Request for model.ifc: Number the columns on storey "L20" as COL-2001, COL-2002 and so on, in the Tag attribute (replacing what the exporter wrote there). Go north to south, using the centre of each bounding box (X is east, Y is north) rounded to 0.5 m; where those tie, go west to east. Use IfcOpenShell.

First a look at what the model holds.

```python
import ifcopenshell
import ifcopenshell.util.element
import ifcopenshell.util.placement

model = ifcopenshell.open("model.ifc")
print(model.schema)
storey = next(s for s in model.by_type("IfcBuildingStorey") if s.Name == "L20")
columns = [e for e in ifcopenshell.util.element.get_decomposition(storey) if e.is_a("IfcColumn")]
for e in sorted(columns, key=lambda e: e.id()):
    origin = ifcopenshell.util.placement.get_local_placement(e.ObjectPlacement)[:3, 3]
    print(e.id(), e.Tag, e.Name, origin.round(2) + 0.0, sep=" | ")
```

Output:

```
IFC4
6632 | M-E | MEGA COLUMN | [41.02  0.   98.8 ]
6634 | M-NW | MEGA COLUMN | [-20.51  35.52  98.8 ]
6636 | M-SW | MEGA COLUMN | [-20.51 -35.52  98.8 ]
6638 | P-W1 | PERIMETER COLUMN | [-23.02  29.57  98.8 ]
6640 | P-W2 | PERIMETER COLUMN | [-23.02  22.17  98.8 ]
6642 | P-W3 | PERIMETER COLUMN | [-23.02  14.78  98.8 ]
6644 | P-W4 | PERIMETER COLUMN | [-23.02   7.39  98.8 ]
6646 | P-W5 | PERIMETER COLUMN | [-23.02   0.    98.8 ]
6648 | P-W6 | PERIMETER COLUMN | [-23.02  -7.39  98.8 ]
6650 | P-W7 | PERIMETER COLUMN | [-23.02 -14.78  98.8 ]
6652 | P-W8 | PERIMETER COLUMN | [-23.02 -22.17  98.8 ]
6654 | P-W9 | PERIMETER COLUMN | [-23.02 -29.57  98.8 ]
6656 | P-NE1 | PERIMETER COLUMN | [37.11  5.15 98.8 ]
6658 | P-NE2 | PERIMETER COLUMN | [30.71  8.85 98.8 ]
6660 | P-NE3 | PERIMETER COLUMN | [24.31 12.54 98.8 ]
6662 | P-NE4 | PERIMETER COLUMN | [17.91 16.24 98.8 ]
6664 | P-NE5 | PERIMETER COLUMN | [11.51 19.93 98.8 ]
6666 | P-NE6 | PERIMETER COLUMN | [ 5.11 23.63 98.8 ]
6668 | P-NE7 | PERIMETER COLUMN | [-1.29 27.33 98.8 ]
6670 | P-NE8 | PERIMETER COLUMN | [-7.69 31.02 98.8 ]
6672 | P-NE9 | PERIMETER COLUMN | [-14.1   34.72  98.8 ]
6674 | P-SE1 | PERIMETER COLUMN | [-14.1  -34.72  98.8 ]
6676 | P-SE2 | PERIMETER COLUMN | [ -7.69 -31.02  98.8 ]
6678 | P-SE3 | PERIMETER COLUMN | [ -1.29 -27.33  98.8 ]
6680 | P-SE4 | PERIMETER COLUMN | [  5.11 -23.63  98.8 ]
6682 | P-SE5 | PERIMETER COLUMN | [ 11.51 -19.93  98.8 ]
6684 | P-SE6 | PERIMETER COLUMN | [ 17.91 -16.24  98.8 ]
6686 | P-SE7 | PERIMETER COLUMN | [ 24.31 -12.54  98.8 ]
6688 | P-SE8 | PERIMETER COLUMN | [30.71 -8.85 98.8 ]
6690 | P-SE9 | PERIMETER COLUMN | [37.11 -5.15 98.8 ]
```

```python
import ifcopenshell
import ifcopenshell.geom
import ifcopenshell.util.element
import ifcopenshell.util.shape

model = ifcopenshell.open("model.ifc")
settings = ifcopenshell.geom.settings()
settings.set("use-world-coords", True)


def centre(element):
    shape = ifcopenshell.geom.create_shape(settings, element)
    return ifcopenshell.util.shape.get_bbox_centroid(shape.geometry)


storey = next(s for s in model.by_type("IfcBuildingStorey") if s.Name == "L20")
columns = [e for e in ifcopenshell.util.element.get_decomposition(storey) if e.is_a("IfcColumn")]

# Insertion points can sit at a corner or the storey origin, so sort by the geometry (in metres).
centres = {e: centre(e) for e in columns}
columns.sort(key=lambda e: (-round(centres[e][1] / 0.5), centres[e][0]))

for i, e in enumerate(columns, start=1):
    number = f"COL-20{i:02d}"
    e.Tag = number
    print(e.id(), number)

model.write("model_rev.ifc")
```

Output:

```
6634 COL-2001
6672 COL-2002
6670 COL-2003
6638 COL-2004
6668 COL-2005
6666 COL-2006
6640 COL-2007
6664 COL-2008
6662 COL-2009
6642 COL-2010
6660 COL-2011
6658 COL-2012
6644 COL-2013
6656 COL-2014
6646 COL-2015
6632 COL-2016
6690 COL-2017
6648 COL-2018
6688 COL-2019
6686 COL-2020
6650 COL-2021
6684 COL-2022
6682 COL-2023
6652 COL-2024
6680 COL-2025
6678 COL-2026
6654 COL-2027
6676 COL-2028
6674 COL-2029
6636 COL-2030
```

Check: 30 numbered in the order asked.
